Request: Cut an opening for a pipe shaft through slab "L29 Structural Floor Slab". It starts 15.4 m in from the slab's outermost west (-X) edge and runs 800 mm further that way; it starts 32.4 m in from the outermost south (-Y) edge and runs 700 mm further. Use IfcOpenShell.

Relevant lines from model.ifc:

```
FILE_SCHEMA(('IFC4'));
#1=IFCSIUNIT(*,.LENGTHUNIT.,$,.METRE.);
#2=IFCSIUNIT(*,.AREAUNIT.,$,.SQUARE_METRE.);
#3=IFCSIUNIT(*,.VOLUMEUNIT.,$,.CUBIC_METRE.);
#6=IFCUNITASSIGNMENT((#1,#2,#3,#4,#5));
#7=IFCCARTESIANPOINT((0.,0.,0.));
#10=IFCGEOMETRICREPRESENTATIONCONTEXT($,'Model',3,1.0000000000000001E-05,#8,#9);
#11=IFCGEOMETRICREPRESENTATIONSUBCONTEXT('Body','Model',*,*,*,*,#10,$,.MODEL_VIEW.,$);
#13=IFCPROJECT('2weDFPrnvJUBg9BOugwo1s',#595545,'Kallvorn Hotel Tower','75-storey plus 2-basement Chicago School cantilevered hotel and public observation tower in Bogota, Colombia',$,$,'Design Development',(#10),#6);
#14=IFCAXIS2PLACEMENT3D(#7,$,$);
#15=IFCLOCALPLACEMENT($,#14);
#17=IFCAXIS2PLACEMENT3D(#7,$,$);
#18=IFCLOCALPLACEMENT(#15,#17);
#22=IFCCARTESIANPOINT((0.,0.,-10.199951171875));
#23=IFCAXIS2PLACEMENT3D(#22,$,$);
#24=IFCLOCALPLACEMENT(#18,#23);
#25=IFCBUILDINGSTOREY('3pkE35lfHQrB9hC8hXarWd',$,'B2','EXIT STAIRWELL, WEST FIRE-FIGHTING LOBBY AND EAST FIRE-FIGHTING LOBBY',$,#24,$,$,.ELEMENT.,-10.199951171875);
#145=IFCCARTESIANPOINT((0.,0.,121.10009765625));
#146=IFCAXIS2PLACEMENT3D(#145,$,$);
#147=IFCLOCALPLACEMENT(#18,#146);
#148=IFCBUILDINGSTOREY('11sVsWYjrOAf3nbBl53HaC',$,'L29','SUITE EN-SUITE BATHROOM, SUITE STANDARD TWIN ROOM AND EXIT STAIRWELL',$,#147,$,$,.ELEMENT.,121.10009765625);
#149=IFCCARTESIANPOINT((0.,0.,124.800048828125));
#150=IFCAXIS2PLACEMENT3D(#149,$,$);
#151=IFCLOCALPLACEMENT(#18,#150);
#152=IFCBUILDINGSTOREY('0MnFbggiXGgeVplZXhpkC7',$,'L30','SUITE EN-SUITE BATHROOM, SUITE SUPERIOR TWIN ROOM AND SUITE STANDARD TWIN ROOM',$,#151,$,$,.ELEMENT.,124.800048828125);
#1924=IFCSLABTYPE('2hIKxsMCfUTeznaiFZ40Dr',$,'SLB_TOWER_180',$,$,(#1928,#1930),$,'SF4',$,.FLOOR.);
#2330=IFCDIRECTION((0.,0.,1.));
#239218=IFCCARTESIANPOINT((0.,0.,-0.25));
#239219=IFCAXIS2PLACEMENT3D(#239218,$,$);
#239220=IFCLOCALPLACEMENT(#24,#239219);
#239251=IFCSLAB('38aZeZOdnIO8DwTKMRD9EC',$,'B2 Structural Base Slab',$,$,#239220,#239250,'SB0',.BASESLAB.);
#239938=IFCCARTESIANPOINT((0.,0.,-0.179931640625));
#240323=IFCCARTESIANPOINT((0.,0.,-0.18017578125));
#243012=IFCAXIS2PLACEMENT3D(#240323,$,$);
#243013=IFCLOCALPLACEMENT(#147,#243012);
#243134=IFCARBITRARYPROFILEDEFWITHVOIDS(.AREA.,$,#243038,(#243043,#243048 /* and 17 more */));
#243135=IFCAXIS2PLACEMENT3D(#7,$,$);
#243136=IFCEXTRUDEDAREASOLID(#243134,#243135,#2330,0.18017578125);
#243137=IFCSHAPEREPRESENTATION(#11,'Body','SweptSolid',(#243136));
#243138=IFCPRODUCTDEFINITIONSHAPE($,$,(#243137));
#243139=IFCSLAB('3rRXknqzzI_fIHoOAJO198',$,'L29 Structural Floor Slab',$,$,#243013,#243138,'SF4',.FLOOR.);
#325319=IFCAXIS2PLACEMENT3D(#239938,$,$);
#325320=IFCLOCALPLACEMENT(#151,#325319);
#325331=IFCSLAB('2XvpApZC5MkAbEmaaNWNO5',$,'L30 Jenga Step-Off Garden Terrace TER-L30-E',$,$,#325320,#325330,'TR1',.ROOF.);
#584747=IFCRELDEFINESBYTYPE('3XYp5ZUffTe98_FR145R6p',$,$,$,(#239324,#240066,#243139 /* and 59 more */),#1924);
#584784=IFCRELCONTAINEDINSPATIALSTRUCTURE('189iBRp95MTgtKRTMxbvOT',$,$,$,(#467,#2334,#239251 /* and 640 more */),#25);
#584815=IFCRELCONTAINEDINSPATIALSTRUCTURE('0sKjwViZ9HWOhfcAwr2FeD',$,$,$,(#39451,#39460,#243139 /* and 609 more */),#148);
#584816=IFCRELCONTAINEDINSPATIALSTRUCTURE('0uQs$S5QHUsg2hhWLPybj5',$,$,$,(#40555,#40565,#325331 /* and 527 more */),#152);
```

```python
import numpy as np
import ifcopenshell
import ifcopenshell.api.feature
import ifcopenshell.api.geometry
import ifcopenshell.api.root
import ifcopenshell.geom
import ifcopenshell.util.placement
import ifcopenshell.util.representation
import ifcopenshell.util.shape
import ifcopenshell.util.unit

model = ifcopenshell.open("model.ifc")
unit_scale = ifcopenshell.util.unit.calculate_unit_scale(model)
settings = ifcopenshell.geom.settings()


def volume(element):
    """Net volume in cubic metres, openings subtracted."""
    shape = ifcopenshell.geom.create_shape(settings, element)
    return ifcopenshell.util.shape.get_volume(shape.geometry)


slab = model.by_id(243139)
before = volume(slab)

# Extent in the slab's own axes, in metres. The edges named are its -X and -Y sides.
slab_shape = ifcopenshell.geom.create_shape(settings, slab)
vertices = ifcopenshell.util.shape.get_vertices(slab_shape.geometry)
x_min, y_min, bottom = vertices.min(axis=0)
top = vertices[:, 2].max()

opening = ifcopenshell.api.root.create_entity(model, ifc_class="IfcOpeningElement", name="Pipe shaft opening", predefined_type="OPENING")
context = ifcopenshell.util.representation.get_context(model, "Model", "Body", "MODEL_VIEW")
width, depth = 0.8, 0.7
outline = [(0.0, 0.0), (width, 0.0), (width, depth), (0.0, depth), (0.0, 0.0)]
# Overshoot both faces by 50 mm so the cut is clean.
shape = ifcopenshell.api.geometry.add_slab_representation(
    model, context=context, depth=top - bottom + 0.1, polyline=outline
)
ifcopenshell.api.geometry.assign_representation(model, product=opening, representation=shape)

matrix = ifcopenshell.util.placement.get_local_placement(slab.ObjectPlacement)
matrix[:, 3] = matrix @ np.append(np.array([x_min + 15.4, y_min + 32.4, bottom - 0.05]) / unit_scale, 1.0)
ifcopenshell.api.geometry.edit_object_placement(model, product=opening, matrix=matrix, is_si=False)
ifcopenshell.api.feature.add_feature(model, feature=opening, element=slab)

after = volume(slab)

print(f"slab volume {before:.3f} -> {after:.3f} m3")

model.write("model_updated.ifc")
```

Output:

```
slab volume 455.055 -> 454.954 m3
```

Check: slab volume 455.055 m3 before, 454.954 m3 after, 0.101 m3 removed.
